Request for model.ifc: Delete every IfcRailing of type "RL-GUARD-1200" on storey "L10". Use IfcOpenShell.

First a look at what the model holds.

```python
import ifcopenshell
import ifcopenshell.util.element

model = ifcopenshell.open("model.ifc")
print(model.schema)
storey = next(s for s in model.by_type("IfcBuildingStorey") if s.Name == "L10")
railings = [e for e in ifcopenshell.util.element.get_decomposition(storey) if e.is_a("IfcRailing")]
seen = {}
for e in railings:
    element_type = ifcopenshell.util.element.get_type(e)
    name = element_type.Name if element_type not in (None, e) else None
    seen[name] = seen.get(name, 0) + 1
for name, count in sorted(seen.items(), key=str):
    print(count, "x", name)
```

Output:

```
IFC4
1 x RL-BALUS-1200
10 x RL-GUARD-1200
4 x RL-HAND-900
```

```python
import ifcopenshell
import ifcopenshell.api.root
import ifcopenshell.util.element

model = ifcopenshell.open("model.ifc")

storey = next(s for s in model.by_type("IfcBuildingStorey") if s.Name == "L10")
railings = [e for e in ifcopenshell.util.element.get_decomposition(storey) if e.is_a("IfcRailing")]
targets = [e for e in railings if (t := ifcopenshell.util.element.get_type(e)) not in (None, e) and t.Name == "RL-GUARD-1200"]

for e in targets:
    ifcopenshell.api.root.remove_product(model, product=e)
print(len(targets), "removed")

model.write("model_v2.ifc")
```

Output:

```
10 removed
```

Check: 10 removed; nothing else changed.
